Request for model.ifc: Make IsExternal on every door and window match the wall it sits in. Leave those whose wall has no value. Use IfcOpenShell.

First a look at what the model holds.

```python
import ifcopenshell
import ifcopenshell.util.element

model = ifcopenshell.open("model.ifc")
print(model.schema)
seen = {}
for e in model.by_type("IfcDoor") + model.by_type("IfcWindow"):
    if not e.FillsVoids:
        continue
    host = e.FillsVoids[0].RelatingOpeningElement.VoidsElements[0].RelatingBuildingElement
    own = ifcopenshell.util.element.get_pset(e, f"Pset_{e.is_a()[3:].removesuffix('StandardCase')}Common", "IsExternal")
    wall = ifcopenshell.util.element.get_pset(host, "Pset_WallCommon", "IsExternal")
    seen[e.is_a(), own, wall] = seen.get((e.is_a(), own, wall), 0) + 1
for (cls, own, wall), count in sorted(seen.items(), key=str):
    print(count, cls, "IsExternal:", own, "| host wall:", wall)
```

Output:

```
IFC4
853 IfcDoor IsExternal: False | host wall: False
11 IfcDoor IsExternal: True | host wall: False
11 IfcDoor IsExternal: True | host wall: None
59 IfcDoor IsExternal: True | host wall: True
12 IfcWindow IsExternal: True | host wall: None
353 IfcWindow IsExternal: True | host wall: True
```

```python
import ifcopenshell
import ifcopenshell.api.pset
import ifcopenshell.util.element

model = ifcopenshell.open("model.ifc")

count = 0
for ifc_class, pset_name in (("IfcDoor", "Pset_DoorCommon"), ("IfcWindow", "Pset_WindowCommon")):
    for e in model.by_type(ifc_class):
        if not e.FillsVoids:
            continue
        host = e.FillsVoids[0].RelatingOpeningElement.VoidsElements[0].RelatingBuildingElement
        external = ifcopenshell.util.element.get_pset(host, "Pset_WallCommon", "IsExternal")
        if external is None or ifcopenshell.util.element.get_pset(e, pset_name, "IsExternal") == external:
            continue
        pset = ifcopenshell.api.pset.add_pset(model, product=e, name=pset_name)
        ifcopenshell.api.pset.edit_pset(model, pset=pset, properties={"IsExternal": external})
        count += 1

print(count, "updated")

model.write("model_updated.ifc")
```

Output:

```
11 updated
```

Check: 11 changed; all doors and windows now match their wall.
